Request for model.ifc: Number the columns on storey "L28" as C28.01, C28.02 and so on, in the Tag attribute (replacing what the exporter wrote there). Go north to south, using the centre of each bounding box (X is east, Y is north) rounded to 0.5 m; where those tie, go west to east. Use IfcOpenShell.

First a look at what the model holds.

```python
import ifcopenshell
import ifcopenshell.util.element
import ifcopenshell.util.placement

model = ifcopenshell.open("model.ifc")
print(model.schema)
storey = next(s for s in model.by_type("IfcBuildingStorey") if s.Name == "L28")
columns = [e for e in ifcopenshell.util.element.get_decomposition(storey) if e.is_a("IfcColumn")]
for e in sorted(columns, key=lambda e: e.id()):
    origin = ifcopenshell.util.placement.get_local_placement(e.ObjectPlacement)[:3, 3]
    print(e.id(), e.Tag, e.Name, origin.round(2) + 0.0, sep=" | ")
```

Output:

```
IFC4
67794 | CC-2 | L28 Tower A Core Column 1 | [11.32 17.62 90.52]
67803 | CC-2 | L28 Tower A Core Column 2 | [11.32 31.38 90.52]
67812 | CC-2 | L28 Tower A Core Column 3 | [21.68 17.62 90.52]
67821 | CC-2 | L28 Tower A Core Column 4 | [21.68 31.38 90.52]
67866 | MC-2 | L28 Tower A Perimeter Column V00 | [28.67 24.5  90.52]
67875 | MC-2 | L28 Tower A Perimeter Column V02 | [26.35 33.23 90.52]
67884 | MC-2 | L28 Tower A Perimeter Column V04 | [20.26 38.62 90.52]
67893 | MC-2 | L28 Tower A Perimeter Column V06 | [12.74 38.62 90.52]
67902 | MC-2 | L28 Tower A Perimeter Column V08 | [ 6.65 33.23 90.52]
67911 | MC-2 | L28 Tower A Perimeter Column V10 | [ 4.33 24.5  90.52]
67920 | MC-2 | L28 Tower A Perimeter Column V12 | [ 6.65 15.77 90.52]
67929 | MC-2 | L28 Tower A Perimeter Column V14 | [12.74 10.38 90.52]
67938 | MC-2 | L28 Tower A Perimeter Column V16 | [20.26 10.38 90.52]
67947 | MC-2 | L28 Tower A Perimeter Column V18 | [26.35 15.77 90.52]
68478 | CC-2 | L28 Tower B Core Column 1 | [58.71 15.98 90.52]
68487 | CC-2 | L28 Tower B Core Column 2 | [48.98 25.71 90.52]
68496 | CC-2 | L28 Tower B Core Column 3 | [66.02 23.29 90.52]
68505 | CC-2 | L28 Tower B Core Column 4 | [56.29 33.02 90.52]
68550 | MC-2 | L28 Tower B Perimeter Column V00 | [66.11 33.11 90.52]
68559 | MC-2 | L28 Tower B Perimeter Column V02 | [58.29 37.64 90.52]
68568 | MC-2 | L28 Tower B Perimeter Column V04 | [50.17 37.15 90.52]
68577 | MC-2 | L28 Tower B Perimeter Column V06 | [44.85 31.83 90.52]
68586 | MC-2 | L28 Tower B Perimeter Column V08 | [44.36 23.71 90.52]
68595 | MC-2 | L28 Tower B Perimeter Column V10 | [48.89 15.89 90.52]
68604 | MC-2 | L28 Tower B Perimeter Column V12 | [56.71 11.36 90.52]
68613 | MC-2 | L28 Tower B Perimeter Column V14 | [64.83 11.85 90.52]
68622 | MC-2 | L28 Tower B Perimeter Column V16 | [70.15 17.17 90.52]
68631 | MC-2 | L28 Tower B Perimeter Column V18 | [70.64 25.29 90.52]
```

```python
import ifcopenshell
import ifcopenshell.geom
import ifcopenshell.util.element
import ifcopenshell.util.shape

model = ifcopenshell.open("model.ifc")
settings = ifcopenshell.geom.settings()
settings.set("use-world-coords", True)


def centre(element):
    shape = ifcopenshell.geom.create_shape(settings, element)
    return ifcopenshell.util.shape.get_bbox_centroid(shape.geometry)


storey = next(s for s in model.by_type("IfcBuildingStorey") if s.Name == "L28")
columns = [e for e in ifcopenshell.util.element.get_decomposition(storey) if e.is_a("IfcColumn")]

# Insertion points can sit at a corner or the storey origin, so sort by the geometry (in metres).
centres = {e: centre(e) for e in columns}
columns.sort(key=lambda e: (-round(centres[e][1] / 0.5), centres[e][0]))

for i, e in enumerate(columns, start=1):
    number = f"C28.{i:02d}"
    e.Tag = number
    print(e.id(), number)

model.write("model_v2.ifc")
```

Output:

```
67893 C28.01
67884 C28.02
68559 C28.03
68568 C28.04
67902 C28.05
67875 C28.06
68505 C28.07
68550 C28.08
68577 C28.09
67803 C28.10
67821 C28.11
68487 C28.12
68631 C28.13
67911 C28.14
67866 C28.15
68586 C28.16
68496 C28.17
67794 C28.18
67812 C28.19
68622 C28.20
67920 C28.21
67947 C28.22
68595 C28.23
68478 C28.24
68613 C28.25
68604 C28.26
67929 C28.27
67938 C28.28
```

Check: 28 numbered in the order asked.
